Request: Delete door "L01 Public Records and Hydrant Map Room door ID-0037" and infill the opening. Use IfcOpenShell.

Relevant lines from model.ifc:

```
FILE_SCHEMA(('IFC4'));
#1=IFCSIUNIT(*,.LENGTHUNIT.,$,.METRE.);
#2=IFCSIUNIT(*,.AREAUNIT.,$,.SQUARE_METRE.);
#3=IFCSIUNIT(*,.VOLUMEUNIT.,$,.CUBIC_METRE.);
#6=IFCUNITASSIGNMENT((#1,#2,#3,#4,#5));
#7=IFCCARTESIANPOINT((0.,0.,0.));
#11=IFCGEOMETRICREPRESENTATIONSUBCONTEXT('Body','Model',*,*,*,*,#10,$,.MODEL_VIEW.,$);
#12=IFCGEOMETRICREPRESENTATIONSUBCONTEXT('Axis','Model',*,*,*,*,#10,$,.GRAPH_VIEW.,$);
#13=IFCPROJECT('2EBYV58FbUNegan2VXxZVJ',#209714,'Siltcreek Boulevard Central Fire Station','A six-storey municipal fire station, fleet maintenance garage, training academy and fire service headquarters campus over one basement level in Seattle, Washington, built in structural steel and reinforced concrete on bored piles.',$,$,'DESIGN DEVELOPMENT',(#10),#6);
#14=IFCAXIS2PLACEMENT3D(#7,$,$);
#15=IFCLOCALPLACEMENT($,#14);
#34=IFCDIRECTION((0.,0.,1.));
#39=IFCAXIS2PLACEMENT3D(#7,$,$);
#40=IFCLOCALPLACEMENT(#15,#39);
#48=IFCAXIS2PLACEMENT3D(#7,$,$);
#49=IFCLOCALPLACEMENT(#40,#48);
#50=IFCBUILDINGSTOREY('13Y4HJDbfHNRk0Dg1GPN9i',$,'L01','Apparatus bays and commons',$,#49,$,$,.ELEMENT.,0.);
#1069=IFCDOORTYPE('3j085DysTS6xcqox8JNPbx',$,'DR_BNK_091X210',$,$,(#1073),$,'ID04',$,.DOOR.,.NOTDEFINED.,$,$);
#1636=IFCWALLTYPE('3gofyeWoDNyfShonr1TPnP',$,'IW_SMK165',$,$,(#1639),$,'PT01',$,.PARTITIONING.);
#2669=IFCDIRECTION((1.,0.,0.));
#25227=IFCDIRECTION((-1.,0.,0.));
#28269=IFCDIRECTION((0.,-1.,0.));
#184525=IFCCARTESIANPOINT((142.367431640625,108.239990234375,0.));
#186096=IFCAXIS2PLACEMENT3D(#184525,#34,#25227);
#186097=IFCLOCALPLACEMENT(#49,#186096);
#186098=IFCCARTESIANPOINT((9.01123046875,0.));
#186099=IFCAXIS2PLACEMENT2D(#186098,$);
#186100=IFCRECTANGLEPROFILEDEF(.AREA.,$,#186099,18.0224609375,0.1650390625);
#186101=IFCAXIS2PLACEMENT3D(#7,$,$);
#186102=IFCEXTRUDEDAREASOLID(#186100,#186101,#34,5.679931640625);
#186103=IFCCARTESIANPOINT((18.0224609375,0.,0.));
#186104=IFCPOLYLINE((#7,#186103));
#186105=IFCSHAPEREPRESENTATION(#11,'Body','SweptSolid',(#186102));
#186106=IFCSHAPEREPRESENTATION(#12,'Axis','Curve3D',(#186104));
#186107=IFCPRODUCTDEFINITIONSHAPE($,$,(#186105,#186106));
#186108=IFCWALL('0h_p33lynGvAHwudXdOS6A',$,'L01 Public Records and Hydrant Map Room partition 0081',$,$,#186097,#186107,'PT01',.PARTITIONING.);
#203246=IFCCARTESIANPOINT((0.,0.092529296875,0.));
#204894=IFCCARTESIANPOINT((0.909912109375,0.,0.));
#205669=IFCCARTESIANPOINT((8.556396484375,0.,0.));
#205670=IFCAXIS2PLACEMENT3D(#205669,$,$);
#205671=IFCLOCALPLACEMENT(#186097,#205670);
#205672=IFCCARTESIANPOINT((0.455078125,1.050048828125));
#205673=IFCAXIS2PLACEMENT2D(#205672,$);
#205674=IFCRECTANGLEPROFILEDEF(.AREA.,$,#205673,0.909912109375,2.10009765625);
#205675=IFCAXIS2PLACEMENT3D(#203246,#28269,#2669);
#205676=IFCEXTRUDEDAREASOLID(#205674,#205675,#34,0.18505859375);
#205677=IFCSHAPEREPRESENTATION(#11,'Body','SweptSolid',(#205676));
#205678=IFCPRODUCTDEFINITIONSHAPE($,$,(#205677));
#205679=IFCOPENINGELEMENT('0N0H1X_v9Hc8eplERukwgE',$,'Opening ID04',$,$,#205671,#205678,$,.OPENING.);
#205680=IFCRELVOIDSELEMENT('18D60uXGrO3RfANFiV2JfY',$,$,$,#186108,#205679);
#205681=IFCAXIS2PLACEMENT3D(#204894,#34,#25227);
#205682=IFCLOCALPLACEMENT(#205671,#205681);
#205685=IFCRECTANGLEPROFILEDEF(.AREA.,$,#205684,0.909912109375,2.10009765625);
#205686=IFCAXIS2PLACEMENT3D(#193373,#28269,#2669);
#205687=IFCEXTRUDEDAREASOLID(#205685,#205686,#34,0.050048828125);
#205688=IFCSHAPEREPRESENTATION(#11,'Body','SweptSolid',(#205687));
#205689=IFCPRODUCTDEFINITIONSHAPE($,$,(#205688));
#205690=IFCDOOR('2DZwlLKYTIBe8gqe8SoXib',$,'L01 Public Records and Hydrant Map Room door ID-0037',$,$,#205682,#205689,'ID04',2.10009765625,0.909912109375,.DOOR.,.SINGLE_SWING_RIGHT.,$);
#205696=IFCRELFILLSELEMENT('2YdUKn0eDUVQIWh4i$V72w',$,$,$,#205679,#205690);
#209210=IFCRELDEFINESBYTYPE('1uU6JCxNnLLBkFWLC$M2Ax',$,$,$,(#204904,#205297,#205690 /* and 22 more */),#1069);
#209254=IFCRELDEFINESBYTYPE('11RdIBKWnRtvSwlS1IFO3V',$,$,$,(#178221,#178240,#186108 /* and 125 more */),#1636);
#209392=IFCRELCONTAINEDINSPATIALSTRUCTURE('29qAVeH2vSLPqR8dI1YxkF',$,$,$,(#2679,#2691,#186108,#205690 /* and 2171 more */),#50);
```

```python
import ifcopenshell
import ifcopenshell.api.feature
import ifcopenshell.api.root
import ifcopenshell.geom
import ifcopenshell.util.shape

model = ifcopenshell.open("model.ifc")
settings = ifcopenshell.geom.settings()


def volume(element):
    """Net volume in cubic metres, openings subtracted."""
    shape = ifcopenshell.geom.create_shape(settings, element)
    return ifcopenshell.util.shape.get_volume(shape.geometry)


door = model.by_guid("2DZwlLKYTIBe8gqe8SoXib")
opening = door.FillsVoids[0].RelatingOpeningElement
wall = opening.VoidsElements[0].RelatingBuildingElement
before = volume(wall)

ifcopenshell.api.root.remove_product(model, product=door)
ifcopenshell.api.feature.remove_feature(model, feature=opening)

after = volume(wall)

print(f"wall volume {before:.3f} -> {after:.3f} m3")

model.write("model_updated.ifc")
```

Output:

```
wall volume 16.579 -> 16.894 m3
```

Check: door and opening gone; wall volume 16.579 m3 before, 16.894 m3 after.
